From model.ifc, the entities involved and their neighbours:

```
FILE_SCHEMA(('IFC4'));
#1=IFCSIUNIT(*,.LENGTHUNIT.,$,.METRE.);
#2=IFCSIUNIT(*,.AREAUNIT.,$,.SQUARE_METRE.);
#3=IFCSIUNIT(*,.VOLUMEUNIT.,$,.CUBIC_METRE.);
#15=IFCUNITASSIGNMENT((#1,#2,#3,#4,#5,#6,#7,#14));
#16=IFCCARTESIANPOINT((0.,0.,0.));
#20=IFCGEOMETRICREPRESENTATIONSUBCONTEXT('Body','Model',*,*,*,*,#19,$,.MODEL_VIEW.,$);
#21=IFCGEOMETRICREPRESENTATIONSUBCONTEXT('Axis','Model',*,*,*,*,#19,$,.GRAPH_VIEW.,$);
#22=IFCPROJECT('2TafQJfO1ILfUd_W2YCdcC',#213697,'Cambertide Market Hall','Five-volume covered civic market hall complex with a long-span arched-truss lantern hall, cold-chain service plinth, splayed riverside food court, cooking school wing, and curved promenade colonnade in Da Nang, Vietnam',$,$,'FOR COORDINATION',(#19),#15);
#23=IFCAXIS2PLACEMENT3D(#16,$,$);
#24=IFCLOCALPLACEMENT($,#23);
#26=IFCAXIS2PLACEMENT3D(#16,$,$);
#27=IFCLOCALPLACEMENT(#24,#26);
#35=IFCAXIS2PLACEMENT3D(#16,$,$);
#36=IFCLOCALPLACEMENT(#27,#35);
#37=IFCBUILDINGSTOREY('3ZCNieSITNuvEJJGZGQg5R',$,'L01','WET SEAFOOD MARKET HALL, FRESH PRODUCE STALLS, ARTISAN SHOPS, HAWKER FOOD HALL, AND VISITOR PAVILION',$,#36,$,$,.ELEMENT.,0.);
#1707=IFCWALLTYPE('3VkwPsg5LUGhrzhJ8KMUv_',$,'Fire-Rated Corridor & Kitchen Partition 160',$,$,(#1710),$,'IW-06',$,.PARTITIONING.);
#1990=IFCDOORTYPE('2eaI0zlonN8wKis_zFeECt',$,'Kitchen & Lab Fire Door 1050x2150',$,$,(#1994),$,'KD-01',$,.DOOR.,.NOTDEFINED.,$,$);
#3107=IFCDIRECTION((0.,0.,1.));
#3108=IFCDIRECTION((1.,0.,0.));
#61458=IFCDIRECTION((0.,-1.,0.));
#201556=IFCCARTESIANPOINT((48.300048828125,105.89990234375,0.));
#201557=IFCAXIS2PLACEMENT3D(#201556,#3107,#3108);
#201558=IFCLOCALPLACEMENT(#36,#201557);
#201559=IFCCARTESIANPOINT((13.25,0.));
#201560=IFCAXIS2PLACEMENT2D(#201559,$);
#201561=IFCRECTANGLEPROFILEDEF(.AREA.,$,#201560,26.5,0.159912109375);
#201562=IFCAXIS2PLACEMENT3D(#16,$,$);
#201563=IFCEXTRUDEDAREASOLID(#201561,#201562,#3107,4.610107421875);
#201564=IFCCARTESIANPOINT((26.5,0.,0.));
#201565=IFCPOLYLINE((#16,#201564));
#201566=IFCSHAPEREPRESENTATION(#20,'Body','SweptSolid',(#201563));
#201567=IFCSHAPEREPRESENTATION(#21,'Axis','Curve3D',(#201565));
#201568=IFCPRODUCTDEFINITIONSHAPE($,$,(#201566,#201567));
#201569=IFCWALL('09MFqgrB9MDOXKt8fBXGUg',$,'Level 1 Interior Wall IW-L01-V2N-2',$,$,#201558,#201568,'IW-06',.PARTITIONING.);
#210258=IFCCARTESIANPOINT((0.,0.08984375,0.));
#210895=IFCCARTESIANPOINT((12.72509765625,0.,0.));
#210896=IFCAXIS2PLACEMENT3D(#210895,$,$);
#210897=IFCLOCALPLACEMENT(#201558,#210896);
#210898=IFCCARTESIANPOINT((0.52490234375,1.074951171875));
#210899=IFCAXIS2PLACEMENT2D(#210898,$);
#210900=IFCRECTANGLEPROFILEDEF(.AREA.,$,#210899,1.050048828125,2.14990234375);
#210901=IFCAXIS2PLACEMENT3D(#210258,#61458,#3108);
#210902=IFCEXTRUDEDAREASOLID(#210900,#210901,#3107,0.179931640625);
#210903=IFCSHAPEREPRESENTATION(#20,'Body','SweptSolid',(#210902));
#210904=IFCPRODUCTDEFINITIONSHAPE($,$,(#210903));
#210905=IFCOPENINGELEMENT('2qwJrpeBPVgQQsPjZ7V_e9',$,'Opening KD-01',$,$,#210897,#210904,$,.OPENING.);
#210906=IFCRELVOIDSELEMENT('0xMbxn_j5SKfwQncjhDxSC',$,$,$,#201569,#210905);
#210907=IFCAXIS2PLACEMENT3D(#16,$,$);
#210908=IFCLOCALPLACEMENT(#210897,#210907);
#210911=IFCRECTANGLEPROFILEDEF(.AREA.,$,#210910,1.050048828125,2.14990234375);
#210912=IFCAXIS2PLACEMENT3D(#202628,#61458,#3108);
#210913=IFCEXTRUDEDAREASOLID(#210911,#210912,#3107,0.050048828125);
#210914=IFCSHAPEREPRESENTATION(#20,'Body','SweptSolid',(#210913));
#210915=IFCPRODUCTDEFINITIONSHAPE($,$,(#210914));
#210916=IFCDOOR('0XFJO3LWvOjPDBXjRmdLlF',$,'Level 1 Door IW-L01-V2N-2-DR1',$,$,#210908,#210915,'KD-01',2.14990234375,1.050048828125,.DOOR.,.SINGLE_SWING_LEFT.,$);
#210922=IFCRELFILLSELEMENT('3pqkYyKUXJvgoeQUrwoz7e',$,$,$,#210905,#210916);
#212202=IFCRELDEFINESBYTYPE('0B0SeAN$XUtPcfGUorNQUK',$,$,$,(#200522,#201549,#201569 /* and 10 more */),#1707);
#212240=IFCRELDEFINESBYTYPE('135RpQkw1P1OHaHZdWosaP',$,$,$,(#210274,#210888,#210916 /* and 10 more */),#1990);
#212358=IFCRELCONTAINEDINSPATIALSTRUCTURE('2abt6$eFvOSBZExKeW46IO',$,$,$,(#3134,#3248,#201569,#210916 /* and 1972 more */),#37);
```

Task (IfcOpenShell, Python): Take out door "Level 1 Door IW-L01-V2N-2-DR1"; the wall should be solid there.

```python
import ifcopenshell
import ifcopenshell.api.feature
import ifcopenshell.api.root
import ifcopenshell.geom
import ifcopenshell.util.shape

model = ifcopenshell.open("model.ifc")
settings = ifcopenshell.geom.settings()


def volume(element):
    """Net volume in cubic metres, openings subtracted."""
    shape = ifcopenshell.geom.create_shape(settings, element)
    return ifcopenshell.util.shape.get_volume(shape.geometry)


door = model.by_guid("0XFJO3LWvOjPDBXjRmdLlF")
opening = door.FillsVoids[0].RelatingOpeningElement
wall = opening.VoidsElements[0].RelatingBuildingElement
before = volume(wall)

ifcopenshell.api.root.remove_product(model, product=door)
ifcopenshell.api.feature.remove_feature(model, feature=opening)

after = volume(wall)

print(f"wall volume {before:.3f} -> {after:.3f} m3")

model.write("model_v2.ifc")
```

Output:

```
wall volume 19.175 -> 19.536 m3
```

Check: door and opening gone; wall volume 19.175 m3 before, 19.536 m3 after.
